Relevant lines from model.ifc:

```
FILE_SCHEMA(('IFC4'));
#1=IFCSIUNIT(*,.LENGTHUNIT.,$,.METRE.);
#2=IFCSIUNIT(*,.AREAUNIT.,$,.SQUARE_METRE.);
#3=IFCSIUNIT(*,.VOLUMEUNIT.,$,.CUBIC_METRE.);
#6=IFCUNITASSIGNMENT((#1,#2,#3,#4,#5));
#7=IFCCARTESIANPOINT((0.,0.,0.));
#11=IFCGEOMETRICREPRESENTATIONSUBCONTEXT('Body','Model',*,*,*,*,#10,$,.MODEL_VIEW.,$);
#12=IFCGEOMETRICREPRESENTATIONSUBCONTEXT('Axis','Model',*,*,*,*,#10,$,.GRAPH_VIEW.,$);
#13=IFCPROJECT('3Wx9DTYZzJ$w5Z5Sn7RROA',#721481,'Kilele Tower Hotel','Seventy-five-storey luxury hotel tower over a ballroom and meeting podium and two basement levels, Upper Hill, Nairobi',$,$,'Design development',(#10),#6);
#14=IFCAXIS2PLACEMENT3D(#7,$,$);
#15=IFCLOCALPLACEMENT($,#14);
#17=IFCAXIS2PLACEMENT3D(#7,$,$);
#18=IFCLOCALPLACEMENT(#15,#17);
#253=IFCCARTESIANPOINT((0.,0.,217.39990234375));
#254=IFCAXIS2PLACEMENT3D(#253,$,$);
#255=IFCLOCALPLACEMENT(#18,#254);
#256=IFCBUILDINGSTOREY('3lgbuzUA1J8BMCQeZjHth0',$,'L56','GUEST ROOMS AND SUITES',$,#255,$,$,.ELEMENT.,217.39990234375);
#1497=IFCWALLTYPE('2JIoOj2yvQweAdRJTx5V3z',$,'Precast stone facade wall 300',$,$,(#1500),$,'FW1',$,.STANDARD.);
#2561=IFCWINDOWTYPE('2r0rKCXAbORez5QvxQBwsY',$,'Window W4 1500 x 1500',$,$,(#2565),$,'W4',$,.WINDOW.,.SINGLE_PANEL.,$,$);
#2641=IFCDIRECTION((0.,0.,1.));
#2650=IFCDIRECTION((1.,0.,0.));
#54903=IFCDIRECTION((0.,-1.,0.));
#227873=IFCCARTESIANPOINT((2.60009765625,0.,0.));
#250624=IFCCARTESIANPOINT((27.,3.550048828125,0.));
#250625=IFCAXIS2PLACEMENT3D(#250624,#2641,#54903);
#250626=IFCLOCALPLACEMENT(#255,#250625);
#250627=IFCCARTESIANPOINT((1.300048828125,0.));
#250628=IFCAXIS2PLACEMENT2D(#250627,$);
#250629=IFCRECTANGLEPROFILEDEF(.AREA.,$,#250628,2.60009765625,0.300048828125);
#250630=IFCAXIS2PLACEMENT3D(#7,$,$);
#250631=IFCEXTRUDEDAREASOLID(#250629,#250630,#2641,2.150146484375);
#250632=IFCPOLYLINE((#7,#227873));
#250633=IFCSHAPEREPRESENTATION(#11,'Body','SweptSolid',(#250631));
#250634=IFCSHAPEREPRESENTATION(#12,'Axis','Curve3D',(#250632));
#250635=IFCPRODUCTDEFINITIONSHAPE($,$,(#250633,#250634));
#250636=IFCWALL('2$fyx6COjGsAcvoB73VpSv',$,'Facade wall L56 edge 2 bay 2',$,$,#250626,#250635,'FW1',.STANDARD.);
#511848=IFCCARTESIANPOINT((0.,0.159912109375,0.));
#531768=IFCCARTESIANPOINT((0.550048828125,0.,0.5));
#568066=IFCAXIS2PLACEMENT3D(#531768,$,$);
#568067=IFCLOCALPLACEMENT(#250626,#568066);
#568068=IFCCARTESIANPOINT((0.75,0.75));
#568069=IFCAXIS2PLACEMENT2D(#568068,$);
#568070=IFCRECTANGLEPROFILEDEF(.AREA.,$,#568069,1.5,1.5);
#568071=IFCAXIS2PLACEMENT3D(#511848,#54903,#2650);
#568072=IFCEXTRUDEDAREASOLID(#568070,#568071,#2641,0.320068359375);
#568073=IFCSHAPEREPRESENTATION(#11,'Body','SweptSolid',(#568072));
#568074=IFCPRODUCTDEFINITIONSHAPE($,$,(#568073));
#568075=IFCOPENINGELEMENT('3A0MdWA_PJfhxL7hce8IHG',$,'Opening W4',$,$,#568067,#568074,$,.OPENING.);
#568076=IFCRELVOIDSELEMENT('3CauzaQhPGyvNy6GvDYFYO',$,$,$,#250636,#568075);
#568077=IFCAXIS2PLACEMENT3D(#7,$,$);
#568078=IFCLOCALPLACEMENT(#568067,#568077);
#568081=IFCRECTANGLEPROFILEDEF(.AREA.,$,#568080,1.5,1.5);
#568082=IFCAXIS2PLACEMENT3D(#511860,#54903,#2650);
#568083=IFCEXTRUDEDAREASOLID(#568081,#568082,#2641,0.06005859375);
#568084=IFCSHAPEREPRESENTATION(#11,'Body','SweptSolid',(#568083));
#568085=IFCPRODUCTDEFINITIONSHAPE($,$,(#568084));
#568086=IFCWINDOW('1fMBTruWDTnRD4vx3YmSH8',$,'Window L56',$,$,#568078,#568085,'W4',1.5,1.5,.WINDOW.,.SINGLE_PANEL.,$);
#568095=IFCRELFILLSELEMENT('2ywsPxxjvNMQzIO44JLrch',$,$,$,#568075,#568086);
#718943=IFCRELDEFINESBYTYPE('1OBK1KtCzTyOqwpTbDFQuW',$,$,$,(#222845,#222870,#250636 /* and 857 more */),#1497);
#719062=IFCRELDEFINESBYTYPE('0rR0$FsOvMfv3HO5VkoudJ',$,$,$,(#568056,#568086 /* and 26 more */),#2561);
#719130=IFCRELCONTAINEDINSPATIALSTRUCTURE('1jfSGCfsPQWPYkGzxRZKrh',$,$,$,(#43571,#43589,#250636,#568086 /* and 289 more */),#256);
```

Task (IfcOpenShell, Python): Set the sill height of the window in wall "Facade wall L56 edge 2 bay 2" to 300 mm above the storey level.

```python
import numpy as np
import ifcopenshell
import ifcopenshell.api.geometry
import ifcopenshell.geom
import ifcopenshell.util.element
import ifcopenshell.util.placement
import ifcopenshell.util.shape
import ifcopenshell.util.unit

model = ifcopenshell.open("model.ifc")
unit_scale = ifcopenshell.util.unit.calculate_unit_scale(model)

window = model.by_id(568086)
opening = window.FillsVoids[0].RelatingOpeningElement
storey = ifcopenshell.util.element.get_container(window, ifc_class="IfcBuildingStorey")
level = ifcopenshell.util.placement.get_local_placement(storey.ObjectPlacement)[2, 3]

# The opening's origin need not be at the sill, so measure its lowest point.
shape = ifcopenshell.geom.create_shape(ifcopenshell.geom.settings(), opening)
bottom = ifcopenshell.util.shape.get_shape_bottom_elevation(shape, shape.geometry) / unit_scale
dz = level + 0.3 / unit_scale - bottom

shift = np.array([0.0, 0.0, dz])
# The window is placed relative to its opening, so it follows when the opening moves.
matrix = ifcopenshell.util.placement.get_local_placement(opening.ObjectPlacement)
matrix[:3, 3] += shift
ifcopenshell.api.geometry.edit_object_placement(
    model, product=opening, matrix=matrix, is_si=False, should_transform_children=True
)

print(f"moved by {dz * unit_scale:+.3f} m")

model.write("model_updated.ifc")
```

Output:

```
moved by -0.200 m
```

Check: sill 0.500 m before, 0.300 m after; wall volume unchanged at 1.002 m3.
